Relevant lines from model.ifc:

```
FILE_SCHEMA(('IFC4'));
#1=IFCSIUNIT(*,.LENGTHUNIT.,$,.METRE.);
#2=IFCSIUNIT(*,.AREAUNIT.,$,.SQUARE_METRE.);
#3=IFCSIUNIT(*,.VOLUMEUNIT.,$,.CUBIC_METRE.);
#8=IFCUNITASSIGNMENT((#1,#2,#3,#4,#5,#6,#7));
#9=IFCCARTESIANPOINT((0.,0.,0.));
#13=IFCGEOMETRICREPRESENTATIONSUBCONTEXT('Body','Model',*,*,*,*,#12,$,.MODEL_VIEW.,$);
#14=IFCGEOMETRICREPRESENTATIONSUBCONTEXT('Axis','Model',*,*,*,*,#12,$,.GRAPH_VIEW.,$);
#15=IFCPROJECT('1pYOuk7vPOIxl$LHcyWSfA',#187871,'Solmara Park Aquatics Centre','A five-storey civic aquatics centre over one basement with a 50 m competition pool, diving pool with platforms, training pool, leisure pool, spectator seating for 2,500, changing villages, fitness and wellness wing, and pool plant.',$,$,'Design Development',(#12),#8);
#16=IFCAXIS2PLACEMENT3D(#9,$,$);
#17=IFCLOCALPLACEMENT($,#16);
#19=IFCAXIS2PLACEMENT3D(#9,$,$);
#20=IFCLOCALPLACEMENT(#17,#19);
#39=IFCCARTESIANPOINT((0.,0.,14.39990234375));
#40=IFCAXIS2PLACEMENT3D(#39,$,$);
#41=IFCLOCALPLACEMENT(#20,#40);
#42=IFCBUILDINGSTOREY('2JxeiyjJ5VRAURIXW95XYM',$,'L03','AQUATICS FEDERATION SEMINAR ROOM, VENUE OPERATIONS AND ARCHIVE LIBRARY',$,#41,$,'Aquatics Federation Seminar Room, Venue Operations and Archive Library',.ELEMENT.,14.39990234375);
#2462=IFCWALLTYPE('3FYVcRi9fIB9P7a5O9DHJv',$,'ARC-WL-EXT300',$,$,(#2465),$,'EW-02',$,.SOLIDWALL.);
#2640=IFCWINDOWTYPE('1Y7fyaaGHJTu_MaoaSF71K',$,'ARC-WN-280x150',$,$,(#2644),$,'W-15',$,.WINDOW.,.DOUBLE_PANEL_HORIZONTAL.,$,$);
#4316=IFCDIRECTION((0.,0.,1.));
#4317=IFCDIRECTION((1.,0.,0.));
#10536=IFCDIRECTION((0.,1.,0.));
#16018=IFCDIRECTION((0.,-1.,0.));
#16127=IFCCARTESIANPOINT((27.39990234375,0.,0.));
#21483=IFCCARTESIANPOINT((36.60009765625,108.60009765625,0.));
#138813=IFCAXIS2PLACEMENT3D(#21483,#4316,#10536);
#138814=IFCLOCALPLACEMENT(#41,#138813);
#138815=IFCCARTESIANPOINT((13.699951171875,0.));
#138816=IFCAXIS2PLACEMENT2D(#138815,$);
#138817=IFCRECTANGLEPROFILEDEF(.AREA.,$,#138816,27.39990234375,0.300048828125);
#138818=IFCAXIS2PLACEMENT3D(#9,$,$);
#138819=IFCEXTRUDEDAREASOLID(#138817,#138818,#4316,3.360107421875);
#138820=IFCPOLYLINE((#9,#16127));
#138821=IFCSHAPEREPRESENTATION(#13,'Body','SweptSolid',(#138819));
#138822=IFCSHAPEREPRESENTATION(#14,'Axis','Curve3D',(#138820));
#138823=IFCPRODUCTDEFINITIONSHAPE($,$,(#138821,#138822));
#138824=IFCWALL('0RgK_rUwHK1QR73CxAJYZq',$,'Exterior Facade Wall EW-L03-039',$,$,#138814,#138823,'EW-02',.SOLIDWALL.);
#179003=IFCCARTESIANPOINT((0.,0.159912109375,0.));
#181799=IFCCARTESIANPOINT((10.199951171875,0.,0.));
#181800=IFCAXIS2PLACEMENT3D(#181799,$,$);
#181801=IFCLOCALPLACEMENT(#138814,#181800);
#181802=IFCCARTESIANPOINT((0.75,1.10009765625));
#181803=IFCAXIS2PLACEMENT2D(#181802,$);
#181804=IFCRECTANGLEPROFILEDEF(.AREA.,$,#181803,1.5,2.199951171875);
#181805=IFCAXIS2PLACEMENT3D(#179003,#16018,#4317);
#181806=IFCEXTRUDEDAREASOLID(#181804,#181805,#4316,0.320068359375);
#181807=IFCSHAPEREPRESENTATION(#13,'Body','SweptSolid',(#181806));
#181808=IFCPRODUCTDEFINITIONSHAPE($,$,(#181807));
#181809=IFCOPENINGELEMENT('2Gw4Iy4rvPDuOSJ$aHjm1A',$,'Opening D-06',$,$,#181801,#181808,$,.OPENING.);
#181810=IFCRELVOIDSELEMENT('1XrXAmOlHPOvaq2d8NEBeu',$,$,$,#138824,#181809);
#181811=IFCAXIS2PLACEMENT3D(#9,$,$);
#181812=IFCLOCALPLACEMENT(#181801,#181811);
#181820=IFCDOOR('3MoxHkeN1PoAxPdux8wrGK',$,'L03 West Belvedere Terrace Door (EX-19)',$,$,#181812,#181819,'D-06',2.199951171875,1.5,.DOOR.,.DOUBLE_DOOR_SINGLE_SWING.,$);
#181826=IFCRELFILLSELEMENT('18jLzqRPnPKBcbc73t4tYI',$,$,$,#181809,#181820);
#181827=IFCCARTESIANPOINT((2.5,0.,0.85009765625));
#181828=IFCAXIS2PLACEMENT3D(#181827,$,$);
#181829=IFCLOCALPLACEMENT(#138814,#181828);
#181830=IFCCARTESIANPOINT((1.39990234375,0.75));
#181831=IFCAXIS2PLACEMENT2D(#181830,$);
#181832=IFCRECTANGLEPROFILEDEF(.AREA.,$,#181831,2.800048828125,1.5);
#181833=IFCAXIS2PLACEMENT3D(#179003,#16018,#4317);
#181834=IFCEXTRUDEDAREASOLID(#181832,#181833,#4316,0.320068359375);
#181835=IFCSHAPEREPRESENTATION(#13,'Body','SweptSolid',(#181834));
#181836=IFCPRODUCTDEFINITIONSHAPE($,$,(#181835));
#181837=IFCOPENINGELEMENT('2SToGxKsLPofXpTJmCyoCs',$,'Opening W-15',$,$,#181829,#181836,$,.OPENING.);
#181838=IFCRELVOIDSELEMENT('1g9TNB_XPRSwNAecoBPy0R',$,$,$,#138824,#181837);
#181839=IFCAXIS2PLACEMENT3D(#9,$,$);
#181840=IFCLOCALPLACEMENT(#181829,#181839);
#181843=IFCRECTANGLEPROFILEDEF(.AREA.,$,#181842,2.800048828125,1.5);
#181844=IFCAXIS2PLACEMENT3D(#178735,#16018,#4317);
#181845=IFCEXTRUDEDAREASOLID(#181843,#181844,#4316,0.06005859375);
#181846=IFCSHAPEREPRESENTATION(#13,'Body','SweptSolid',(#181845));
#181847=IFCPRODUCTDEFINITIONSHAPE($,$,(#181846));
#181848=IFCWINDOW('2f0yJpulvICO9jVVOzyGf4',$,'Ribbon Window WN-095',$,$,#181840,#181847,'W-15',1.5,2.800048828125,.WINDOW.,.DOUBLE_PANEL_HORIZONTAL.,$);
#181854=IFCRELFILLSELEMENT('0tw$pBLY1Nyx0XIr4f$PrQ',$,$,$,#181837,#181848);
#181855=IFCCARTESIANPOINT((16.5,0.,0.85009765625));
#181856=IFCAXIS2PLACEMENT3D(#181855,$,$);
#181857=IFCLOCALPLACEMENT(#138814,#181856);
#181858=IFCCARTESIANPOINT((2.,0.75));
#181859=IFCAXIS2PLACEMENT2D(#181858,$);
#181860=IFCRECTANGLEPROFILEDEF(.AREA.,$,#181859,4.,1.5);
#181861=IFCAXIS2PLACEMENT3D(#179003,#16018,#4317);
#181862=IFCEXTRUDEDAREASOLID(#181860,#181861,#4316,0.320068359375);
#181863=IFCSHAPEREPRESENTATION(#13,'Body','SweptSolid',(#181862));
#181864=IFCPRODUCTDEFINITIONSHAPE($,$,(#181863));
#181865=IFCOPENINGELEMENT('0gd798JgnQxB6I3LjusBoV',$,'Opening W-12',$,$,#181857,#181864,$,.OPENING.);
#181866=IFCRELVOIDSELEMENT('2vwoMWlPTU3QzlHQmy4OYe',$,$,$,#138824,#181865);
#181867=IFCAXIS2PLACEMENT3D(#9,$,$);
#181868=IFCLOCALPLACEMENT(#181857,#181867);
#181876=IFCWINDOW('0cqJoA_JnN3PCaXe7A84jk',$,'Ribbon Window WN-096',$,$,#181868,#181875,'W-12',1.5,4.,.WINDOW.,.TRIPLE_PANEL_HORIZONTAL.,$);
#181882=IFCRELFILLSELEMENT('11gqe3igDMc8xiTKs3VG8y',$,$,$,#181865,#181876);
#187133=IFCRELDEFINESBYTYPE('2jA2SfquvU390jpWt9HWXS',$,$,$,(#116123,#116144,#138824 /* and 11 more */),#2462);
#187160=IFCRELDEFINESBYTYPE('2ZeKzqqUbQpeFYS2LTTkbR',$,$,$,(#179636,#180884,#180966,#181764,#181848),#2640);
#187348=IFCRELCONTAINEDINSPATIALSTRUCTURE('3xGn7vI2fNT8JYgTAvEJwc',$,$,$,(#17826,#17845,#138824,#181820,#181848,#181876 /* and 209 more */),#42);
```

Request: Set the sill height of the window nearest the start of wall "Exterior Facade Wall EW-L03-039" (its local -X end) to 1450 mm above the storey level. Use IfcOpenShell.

```python
import numpy as np
import ifcopenshell
import ifcopenshell.api.geometry
import ifcopenshell.geom
import ifcopenshell.util.element
import ifcopenshell.util.placement
import ifcopenshell.util.shape
import ifcopenshell.util.unit

model = ifcopenshell.open("model.ifc")
unit_scale = ifcopenshell.util.unit.calculate_unit_scale(model)

window = model.by_guid("2f0yJpulvICO9jVVOzyGf4")
opening = window.FillsVoids[0].RelatingOpeningElement
storey = ifcopenshell.util.element.get_container(window, ifc_class="IfcBuildingStorey")
level = ifcopenshell.util.placement.get_local_placement(storey.ObjectPlacement)[2, 3]

# The opening's origin need not be at the sill, so measure its lowest point.
shape = ifcopenshell.geom.create_shape(ifcopenshell.geom.settings(), opening)
bottom = ifcopenshell.util.shape.get_shape_bottom_elevation(shape, shape.geometry) / unit_scale
dz = level + 1.45 / unit_scale - bottom

shift = np.array([0.0, 0.0, dz])
# The window is placed relative to its opening, so it follows when the opening moves.
matrix = ifcopenshell.util.placement.get_local_placement(opening.ObjectPlacement)
matrix[:3, 3] += shift
ifcopenshell.api.geometry.edit_object_placement(
    model, product=opening, matrix=matrix, is_si=False, should_transform_children=True
)

print(f"moved by {dz * unit_scale:+.3f} m")

model.write("model_rev.ifc")
```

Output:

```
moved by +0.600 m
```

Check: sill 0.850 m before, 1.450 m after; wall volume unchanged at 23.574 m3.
